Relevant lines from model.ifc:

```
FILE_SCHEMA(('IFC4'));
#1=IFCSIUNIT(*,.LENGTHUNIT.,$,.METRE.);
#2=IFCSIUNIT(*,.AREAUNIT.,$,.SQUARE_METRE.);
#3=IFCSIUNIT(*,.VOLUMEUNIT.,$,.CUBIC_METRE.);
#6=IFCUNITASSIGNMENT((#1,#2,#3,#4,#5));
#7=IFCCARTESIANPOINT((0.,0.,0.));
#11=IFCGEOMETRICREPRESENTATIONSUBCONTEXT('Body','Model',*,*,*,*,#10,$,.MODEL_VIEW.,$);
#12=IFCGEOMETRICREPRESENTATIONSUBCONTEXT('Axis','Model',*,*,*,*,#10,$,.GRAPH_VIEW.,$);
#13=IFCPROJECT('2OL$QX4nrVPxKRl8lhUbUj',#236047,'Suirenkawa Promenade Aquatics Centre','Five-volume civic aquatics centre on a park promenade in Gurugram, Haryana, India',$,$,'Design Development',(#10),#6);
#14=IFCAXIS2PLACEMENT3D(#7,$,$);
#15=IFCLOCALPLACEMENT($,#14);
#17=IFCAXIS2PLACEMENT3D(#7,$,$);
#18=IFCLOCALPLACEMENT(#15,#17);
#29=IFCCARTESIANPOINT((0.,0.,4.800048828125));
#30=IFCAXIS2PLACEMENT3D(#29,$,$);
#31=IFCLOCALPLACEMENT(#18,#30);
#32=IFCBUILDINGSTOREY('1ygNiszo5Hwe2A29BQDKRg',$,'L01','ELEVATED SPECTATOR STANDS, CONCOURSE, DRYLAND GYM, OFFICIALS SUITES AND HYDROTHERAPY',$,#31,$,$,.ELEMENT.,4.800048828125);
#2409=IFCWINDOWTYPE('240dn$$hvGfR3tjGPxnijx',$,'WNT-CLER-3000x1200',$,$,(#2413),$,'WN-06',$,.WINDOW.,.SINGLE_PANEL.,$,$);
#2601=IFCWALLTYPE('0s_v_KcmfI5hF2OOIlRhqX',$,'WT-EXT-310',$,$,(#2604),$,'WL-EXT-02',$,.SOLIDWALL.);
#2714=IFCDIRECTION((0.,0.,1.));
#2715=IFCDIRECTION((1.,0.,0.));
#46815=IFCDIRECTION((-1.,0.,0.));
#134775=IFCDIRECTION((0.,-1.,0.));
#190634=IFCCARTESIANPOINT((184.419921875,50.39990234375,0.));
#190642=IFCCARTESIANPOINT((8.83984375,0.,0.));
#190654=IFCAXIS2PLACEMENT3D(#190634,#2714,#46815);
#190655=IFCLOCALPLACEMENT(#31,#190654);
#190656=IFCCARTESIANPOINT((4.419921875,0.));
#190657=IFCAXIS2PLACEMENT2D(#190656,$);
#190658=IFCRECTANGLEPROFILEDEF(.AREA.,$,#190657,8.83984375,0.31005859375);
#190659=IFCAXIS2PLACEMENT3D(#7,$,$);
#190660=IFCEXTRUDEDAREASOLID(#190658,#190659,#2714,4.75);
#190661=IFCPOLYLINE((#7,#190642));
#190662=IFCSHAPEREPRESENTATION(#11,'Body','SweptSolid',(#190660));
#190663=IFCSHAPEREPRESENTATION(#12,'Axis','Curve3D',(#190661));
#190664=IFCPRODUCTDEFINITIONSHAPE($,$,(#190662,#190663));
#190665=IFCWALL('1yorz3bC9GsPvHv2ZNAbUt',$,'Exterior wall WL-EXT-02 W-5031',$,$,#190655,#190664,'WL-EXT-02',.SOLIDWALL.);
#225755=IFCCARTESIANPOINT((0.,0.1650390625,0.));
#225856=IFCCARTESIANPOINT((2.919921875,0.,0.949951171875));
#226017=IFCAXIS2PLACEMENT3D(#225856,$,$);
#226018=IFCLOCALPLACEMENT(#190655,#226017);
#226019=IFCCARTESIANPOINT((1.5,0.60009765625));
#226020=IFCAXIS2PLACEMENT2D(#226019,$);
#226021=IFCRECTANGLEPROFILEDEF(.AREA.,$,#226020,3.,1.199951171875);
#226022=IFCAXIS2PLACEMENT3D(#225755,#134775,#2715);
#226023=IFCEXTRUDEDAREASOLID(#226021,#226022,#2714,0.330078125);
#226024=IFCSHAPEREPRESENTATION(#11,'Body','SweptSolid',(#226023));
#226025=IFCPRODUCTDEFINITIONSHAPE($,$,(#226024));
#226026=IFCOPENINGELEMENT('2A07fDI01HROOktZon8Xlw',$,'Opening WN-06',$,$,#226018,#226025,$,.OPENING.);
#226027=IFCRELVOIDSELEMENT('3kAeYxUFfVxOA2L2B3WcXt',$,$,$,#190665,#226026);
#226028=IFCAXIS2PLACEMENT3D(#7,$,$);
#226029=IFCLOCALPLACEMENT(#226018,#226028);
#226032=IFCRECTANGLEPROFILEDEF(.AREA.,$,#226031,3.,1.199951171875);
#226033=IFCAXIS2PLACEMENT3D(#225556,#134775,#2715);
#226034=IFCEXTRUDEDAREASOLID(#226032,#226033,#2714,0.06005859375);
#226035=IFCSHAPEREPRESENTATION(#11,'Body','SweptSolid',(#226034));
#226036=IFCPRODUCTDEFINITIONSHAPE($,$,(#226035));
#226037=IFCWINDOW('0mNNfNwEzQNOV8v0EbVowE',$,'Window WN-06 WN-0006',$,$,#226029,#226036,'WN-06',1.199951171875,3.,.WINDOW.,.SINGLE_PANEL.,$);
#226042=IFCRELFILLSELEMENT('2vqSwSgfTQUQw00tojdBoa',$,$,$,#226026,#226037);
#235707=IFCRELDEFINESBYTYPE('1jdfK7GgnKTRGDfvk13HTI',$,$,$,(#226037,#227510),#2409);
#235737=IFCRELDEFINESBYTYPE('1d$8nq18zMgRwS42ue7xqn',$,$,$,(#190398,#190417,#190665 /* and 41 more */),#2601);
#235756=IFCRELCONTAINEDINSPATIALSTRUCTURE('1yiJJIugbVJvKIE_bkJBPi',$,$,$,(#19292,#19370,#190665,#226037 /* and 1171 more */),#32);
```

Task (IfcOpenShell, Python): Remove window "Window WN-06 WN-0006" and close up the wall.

```python
import ifcopenshell
import ifcopenshell.api.feature
import ifcopenshell.api.root
import ifcopenshell.geom
import ifcopenshell.util.shape

model = ifcopenshell.open("model.ifc")
settings = ifcopenshell.geom.settings()


def volume(element):
    """Net volume in cubic metres, openings subtracted."""
    shape = ifcopenshell.geom.create_shape(settings, element)
    return ifcopenshell.util.shape.get_volume(shape.geometry)


window = model.by_guid("0mNNfNwEzQNOV8v0EbVowE")
opening = window.FillsVoids[0].RelatingOpeningElement
wall = opening.VoidsElements[0].RelatingBuildingElement
before = volume(wall)

ifcopenshell.api.root.remove_product(model, product=window)
ifcopenshell.api.feature.remove_feature(model, feature=opening)

after = volume(wall)

print(f"wall volume {before:.3f} -> {after:.3f} m3")

model.write("model_v2.ifc")
```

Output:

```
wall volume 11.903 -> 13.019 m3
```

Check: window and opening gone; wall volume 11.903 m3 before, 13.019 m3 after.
